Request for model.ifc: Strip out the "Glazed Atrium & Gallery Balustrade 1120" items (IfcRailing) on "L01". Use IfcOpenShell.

First a look at what the model holds.

```python
import ifcopenshell
import ifcopenshell.util.element

model = ifcopenshell.open("model.ifc")
print(model.schema)
storey = next(s for s in model.by_type("IfcBuildingStorey") if s.Name == "L01")
railings = [e for e in ifcopenshell.util.element.get_decomposition(storey) if e.is_a("IfcRailing")]
seen = {}
for e in railings:
    element_type = ifcopenshell.util.element.get_type(e)
    name = element_type.Name if element_type not in (None, e) else None
    seen[name] = seen.get(name, 0) + 1
for name, count in sorted(seen.items(), key=str):
    print(count, "x", name)
```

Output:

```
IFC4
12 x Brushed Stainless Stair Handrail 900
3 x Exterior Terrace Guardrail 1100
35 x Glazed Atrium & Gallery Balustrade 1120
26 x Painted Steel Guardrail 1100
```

```python
import ifcopenshell
import ifcopenshell.api.root
import ifcopenshell.util.element

model = ifcopenshell.open("model.ifc")

storey = next(s for s in model.by_type("IfcBuildingStorey") if s.Name == "L01")
railings = [e for e in ifcopenshell.util.element.get_decomposition(storey) if e.is_a("IfcRailing")]
targets = [e for e in railings if (t := ifcopenshell.util.element.get_type(e)) not in (None, e) and t.Name == "Glazed Atrium & Gallery Balustrade 1120"]

for e in targets:
    ifcopenshell.api.root.remove_product(model, product=e)
print(len(targets), "removed")

model.write("model_updated.ifc")
```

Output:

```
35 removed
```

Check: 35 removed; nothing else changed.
